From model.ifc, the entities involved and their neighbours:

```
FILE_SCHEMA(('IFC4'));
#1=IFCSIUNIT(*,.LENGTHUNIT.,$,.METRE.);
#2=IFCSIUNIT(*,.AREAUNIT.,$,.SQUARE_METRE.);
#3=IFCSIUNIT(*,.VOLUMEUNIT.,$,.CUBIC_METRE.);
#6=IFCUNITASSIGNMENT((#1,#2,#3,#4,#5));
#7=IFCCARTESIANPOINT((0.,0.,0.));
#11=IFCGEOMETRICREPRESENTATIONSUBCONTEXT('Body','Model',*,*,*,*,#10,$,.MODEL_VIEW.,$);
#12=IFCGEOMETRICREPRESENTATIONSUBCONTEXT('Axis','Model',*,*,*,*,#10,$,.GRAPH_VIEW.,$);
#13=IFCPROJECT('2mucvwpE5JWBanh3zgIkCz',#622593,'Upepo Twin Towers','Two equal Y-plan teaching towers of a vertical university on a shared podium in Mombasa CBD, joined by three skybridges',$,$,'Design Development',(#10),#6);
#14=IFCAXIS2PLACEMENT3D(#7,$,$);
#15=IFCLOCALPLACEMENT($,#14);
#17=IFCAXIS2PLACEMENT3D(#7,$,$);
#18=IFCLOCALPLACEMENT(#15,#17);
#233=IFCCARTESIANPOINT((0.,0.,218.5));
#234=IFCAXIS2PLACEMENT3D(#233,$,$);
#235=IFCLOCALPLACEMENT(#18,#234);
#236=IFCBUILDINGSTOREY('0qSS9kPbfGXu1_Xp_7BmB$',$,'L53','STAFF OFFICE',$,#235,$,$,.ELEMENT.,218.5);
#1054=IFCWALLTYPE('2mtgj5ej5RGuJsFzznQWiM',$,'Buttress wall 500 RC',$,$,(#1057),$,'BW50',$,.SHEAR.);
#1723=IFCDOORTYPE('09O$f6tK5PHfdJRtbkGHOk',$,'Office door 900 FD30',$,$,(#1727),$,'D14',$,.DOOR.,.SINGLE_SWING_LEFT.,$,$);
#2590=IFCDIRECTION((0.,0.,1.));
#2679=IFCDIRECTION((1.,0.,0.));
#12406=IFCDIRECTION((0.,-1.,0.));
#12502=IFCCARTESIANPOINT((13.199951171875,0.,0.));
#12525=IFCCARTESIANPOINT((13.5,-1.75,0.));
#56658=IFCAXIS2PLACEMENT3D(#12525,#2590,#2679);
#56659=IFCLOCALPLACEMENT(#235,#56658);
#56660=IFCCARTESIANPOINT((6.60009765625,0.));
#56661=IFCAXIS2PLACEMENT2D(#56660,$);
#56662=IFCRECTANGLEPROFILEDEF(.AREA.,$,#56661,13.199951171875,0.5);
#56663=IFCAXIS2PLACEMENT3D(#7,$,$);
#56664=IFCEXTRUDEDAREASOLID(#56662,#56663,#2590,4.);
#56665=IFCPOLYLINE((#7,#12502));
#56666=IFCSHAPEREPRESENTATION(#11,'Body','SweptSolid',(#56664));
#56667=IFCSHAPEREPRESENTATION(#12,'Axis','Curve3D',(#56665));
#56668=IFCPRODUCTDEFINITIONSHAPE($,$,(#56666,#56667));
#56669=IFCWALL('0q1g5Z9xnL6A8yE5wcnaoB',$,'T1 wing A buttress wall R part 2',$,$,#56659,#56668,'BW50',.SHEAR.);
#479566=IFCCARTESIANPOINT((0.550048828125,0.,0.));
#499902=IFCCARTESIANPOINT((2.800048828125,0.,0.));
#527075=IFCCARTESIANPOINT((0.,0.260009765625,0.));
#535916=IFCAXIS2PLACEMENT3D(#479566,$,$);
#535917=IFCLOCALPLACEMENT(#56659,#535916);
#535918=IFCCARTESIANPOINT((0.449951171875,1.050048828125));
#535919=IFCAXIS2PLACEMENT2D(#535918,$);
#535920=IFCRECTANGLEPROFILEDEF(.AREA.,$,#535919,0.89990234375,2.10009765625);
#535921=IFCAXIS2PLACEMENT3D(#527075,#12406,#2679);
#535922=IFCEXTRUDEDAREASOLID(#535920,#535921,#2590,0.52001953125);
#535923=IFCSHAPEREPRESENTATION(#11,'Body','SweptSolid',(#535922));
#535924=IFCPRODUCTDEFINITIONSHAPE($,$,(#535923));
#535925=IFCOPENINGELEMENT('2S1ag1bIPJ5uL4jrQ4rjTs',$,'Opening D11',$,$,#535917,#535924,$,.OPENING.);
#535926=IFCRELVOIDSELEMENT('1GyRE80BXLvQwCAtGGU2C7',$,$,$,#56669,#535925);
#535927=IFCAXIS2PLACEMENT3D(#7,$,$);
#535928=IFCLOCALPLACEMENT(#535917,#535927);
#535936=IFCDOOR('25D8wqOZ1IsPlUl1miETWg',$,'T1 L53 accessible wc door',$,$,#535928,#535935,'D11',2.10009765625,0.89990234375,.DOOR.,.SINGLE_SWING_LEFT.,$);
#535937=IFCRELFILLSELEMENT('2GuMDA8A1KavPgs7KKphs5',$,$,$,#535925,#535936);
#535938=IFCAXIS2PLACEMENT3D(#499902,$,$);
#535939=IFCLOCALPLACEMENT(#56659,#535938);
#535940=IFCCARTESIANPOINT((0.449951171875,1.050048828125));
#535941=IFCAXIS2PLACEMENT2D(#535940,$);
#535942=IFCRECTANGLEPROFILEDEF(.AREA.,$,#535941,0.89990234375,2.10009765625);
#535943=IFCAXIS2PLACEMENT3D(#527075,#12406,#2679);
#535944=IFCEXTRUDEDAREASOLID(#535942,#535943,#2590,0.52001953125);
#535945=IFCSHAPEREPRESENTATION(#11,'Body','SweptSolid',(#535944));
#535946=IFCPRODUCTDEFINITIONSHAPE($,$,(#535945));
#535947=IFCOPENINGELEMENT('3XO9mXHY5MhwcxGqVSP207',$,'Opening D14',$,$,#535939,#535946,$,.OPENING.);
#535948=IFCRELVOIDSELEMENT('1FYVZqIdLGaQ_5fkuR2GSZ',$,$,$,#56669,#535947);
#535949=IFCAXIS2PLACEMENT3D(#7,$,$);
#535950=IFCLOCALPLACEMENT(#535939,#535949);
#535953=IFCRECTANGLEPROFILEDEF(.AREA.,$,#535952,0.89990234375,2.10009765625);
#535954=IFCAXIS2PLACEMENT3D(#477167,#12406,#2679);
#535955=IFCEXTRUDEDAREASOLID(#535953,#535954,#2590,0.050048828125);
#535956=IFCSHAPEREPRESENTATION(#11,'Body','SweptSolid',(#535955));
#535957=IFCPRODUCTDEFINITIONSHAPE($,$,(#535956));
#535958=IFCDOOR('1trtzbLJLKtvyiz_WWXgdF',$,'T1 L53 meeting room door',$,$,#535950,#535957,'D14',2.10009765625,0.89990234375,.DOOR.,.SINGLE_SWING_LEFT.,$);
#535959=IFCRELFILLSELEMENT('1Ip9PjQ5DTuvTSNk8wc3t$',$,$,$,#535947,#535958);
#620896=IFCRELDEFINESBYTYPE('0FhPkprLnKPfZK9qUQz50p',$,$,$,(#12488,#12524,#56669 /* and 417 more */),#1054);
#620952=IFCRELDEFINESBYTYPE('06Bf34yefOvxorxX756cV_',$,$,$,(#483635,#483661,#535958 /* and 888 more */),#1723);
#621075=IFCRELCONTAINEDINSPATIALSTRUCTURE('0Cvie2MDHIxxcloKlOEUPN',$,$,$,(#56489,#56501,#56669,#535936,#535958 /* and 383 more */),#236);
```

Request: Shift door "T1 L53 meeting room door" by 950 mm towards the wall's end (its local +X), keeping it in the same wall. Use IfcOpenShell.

```python
import ifcopenshell
import ifcopenshell.api.geometry
import ifcopenshell.util.placement

model = ifcopenshell.open("model.ifc")

door = model.by_id(535958)
opening = door.FillsVoids[0].RelatingOpeningElement
wall = opening.VoidsElements[0].RelatingBuildingElement

wall_matrix = ifcopenshell.util.placement.get_local_placement(wall.ObjectPlacement)
shift = wall_matrix[:3, 0] * 0.95
before = ifcopenshell.util.placement.get_local_placement(door.ObjectPlacement)[:3, 3].copy()

# The door is placed relative to its opening, so it follows when the opening moves.
matrix = ifcopenshell.util.placement.get_local_placement(opening.ObjectPlacement)
matrix[:3, 3] += shift
ifcopenshell.api.geometry.edit_object_placement(
    model, product=opening, matrix=matrix, is_si=False, should_transform_children=True
)

after = ifcopenshell.util.placement.get_local_placement(door.ObjectPlacement)[:3, 3]
print("door moved by", (after - before).round(3) + 0.0)

model.write("model_rev.ifc")
```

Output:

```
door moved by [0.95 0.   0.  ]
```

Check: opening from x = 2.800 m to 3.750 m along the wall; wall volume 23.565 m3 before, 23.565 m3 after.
